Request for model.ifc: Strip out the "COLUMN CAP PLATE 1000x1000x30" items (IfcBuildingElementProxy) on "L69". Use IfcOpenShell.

First a look at what the model holds.

```python
import ifcopenshell
import ifcopenshell.util.element

model = ifcopenshell.open("model.ifc")
print(model.schema)
storey = next(s for s in model.by_type("IfcBuildingStorey") if s.Name == "L69")
proxies = [e for e in ifcopenshell.util.element.get_decomposition(storey) if e.is_a("IfcBuildingElementProxy")]
seen = {}
for e in proxies:
    element_type = ifcopenshell.util.element.get_type(e)
    name = element_type.Name if element_type not in (None, e) else None
    seen[name] = seen.get(name, 0) + 1
for name, count in sorted(seen.items(), key=str):
    print(count, "x", name)
```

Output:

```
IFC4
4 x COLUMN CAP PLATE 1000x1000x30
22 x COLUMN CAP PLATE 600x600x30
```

```python
import ifcopenshell
import ifcopenshell.api.root
import ifcopenshell.util.element

model = ifcopenshell.open("model.ifc")

storey = next(s for s in model.by_type("IfcBuildingStorey") if s.Name == "L69")
proxies = [e for e in ifcopenshell.util.element.get_decomposition(storey) if e.is_a("IfcBuildingElementProxy")]
targets = [e for e in proxies if (t := ifcopenshell.util.element.get_type(e)) not in (None, e) and t.Name == "COLUMN CAP PLATE 1000x1000x30"]

for e in targets:
    ifcopenshell.api.root.remove_product(model, product=e)
print(len(targets), "removed")

model.write("model_v2.ifc")
```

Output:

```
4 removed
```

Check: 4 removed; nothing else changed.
